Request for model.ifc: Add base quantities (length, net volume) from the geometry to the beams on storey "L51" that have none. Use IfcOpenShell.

First a look at what the model holds.

```python
import ifcopenshell
import ifcopenshell.util.element
import ifcopenshell.util.unit

model = ifcopenshell.open("model.ifc")
print(model.schema)
for unit_type in ("LENGTHUNIT", "AREAUNIT", "VOLUMEUNIT"):
    print(unit_type, ifcopenshell.util.unit.calculate_unit_scale(model, unit_type))
storey = next(s for s in model.by_type("IfcBuildingStorey") if s.Name == "L51")
beams = [e for e in ifcopenshell.util.element.get_decomposition(storey) if e.is_a("IfcBeam")]
for e in sorted(beams, key=lambda e: e.id()):
    print(e.id(), e.is_a(), e.Name, list(ifcopenshell.util.element.get_psets(e, qtos_only=True)), sep=" | ")
```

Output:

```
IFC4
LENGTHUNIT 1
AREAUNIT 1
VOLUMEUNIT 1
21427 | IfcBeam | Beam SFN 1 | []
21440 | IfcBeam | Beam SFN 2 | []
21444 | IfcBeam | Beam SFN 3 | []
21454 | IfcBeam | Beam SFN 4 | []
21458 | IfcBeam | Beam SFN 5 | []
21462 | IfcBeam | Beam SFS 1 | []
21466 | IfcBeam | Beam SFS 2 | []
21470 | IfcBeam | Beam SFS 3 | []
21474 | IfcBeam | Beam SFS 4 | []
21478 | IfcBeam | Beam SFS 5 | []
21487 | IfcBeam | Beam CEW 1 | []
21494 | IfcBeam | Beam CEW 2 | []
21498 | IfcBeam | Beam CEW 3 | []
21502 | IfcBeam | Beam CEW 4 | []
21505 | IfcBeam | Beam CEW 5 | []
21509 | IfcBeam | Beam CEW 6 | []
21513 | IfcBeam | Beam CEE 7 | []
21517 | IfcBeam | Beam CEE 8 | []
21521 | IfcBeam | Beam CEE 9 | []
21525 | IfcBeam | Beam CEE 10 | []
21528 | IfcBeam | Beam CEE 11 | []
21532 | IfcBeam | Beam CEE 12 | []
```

```python
import ifcopenshell
import ifcopenshell.api.pset
import ifcopenshell.geom
import ifcopenshell.util.element
import ifcopenshell.util.shape
import ifcopenshell.util.unit

model = ifcopenshell.open("model.ifc")
unit_scale = ifcopenshell.util.unit.calculate_unit_scale(model)
volume_scale = ifcopenshell.util.unit.calculate_unit_scale(model, "VOLUMEUNIT")
settings = ifcopenshell.geom.settings()

storey = next(s for s in model.by_type("IfcBuildingStorey") if s.Name == "L51")
beams = [e for e in ifcopenshell.util.element.get_decomposition(storey) if e.is_a("IfcBeam")]

for e in sorted(beams, key=lambda e: e.id()):
    if ifcopenshell.util.element.get_psets(e, qtos_only=True, should_inherit=False):
        continue
    # Geometry comes back in metres, in the element's own axes.
    shape = ifcopenshell.geom.create_shape(settings, e)
    values = {
        "Length": ifcopenshell.util.shape.get_max_xyz(shape.geometry) / unit_scale,
        "NetVolume": ifcopenshell.util.shape.get_volume(shape.geometry) / volume_scale,
    }
    qto = ifcopenshell.api.pset.add_qto(model, product=e, name="Qto_BeamBaseQuantities")
    ifcopenshell.api.pset.edit_qto(model, qto=qto, properties=values)
    print(e.id(), {k: round(v, 3) for k, v in values.items()})

model.write("model_v2.ifc")
```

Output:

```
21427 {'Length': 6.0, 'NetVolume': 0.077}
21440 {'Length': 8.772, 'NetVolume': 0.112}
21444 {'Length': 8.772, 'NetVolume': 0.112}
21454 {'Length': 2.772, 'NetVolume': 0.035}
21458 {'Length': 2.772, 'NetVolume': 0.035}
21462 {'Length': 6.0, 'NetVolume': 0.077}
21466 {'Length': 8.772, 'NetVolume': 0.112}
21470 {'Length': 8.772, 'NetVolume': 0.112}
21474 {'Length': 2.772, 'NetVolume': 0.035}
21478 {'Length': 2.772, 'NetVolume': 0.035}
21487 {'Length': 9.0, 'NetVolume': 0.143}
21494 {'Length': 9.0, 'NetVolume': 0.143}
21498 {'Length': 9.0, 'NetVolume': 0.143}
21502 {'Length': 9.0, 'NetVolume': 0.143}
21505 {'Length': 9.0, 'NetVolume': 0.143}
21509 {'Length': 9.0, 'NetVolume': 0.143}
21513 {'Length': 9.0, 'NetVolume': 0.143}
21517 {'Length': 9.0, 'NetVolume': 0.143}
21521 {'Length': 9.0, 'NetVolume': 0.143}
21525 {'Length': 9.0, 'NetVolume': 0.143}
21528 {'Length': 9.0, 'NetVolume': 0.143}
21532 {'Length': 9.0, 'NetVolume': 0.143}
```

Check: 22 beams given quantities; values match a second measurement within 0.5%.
